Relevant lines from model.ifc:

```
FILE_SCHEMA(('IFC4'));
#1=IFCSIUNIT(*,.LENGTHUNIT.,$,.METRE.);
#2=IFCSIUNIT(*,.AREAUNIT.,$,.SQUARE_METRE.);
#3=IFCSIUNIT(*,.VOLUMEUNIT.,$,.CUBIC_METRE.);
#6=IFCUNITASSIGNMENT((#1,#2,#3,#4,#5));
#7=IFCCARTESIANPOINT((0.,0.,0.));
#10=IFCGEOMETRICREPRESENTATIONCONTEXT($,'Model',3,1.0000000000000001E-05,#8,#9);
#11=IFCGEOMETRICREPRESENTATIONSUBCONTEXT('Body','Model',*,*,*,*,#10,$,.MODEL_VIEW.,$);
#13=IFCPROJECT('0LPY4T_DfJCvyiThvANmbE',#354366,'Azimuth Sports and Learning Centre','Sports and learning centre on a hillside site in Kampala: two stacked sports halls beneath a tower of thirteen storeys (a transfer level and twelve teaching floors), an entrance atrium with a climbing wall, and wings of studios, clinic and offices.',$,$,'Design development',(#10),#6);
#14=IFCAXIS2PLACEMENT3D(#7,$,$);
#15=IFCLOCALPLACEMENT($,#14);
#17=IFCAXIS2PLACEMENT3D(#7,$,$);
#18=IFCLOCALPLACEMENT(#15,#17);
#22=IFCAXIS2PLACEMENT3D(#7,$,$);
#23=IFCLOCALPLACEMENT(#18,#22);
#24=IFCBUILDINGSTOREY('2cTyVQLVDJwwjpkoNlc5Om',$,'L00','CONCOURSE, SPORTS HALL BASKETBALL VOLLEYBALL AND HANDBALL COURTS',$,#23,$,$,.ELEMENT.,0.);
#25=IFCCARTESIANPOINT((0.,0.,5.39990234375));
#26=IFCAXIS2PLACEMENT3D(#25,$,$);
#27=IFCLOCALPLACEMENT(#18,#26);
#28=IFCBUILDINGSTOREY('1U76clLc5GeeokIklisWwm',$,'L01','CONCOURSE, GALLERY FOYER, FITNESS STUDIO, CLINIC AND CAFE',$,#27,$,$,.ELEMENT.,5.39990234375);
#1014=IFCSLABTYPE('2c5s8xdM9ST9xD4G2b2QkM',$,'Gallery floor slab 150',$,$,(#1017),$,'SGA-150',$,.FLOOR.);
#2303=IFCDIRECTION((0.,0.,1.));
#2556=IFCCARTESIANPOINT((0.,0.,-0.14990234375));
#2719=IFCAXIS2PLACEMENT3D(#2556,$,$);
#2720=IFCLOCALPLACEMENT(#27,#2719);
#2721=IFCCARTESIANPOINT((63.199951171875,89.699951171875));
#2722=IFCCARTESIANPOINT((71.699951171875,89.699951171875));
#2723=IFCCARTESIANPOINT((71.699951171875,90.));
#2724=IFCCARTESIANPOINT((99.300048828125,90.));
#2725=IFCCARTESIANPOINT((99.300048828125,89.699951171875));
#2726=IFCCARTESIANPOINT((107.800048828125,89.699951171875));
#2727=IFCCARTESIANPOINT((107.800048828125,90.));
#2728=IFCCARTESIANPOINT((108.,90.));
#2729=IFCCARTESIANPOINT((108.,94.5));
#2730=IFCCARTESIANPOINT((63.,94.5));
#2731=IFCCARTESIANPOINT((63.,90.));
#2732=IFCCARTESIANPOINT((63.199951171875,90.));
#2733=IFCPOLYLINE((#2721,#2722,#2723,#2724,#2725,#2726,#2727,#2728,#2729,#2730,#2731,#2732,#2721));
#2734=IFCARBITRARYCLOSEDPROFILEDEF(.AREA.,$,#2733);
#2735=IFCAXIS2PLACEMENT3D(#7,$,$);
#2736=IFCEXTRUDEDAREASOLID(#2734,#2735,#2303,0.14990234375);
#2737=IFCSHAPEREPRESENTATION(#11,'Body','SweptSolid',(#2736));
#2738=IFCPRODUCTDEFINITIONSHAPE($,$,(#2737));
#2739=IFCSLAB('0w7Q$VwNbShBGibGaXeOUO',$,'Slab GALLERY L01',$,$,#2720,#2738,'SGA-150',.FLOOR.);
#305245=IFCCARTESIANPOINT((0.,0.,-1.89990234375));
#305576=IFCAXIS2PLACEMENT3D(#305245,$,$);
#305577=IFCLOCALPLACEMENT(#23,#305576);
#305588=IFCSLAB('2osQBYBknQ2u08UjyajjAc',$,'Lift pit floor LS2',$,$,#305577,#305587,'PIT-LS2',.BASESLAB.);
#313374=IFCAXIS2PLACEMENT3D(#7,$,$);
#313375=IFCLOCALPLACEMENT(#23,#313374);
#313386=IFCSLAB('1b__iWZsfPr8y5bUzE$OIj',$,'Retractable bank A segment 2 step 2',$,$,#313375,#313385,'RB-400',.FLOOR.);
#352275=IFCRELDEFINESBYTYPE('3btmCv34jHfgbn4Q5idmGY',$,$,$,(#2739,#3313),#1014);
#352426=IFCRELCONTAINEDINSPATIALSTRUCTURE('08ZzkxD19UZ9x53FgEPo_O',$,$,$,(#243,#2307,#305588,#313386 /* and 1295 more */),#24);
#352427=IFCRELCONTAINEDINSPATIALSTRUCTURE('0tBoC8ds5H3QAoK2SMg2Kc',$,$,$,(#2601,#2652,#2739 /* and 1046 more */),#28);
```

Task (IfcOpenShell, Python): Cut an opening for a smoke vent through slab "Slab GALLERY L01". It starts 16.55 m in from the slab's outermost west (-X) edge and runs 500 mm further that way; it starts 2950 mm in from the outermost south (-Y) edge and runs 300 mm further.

```python
import numpy as np
import ifcopenshell
import ifcopenshell.api.feature
import ifcopenshell.api.geometry
import ifcopenshell.api.root
import ifcopenshell.geom
import ifcopenshell.util.placement
import ifcopenshell.util.representation
import ifcopenshell.util.shape
import ifcopenshell.util.unit

model = ifcopenshell.open("model.ifc")
unit_scale = ifcopenshell.util.unit.calculate_unit_scale(model)
settings = ifcopenshell.geom.settings()


def volume(element):
    """Net volume in cubic metres, openings subtracted."""
    shape = ifcopenshell.geom.create_shape(settings, element)
    return ifcopenshell.util.shape.get_volume(shape.geometry)


slab = model.by_guid("0w7Q$VwNbShBGibGaXeOUO")
before = volume(slab)

# Extent in the slab's own axes, in metres. The edges named are its -X and -Y sides.
slab_shape = ifcopenshell.geom.create_shape(settings, slab)
vertices = ifcopenshell.util.shape.get_vertices(slab_shape.geometry)
x_min, y_min, bottom = vertices.min(axis=0)
top = vertices[:, 2].max()

opening = ifcopenshell.api.root.create_entity(model, ifc_class="IfcOpeningElement", name="Smoke vent opening", predefined_type="OPENING")
context = ifcopenshell.util.representation.get_context(model, "Model", "Body", "MODEL_VIEW")
width, depth = 0.5, 0.3
outline = [(0.0, 0.0), (width, 0.0), (width, depth), (0.0, depth), (0.0, 0.0)]
# Overshoot both faces by 50 mm so the cut is clean.
shape = ifcopenshell.api.geometry.add_slab_representation(
    model, context=context, depth=top - bottom + 0.1, polyline=outline
)
ifcopenshell.api.geometry.assign_representation(model, product=opening, representation=shape)

matrix = ifcopenshell.util.placement.get_local_placement(slab.ObjectPlacement)
matrix[:, 3] = matrix @ np.append(np.array([x_min + 16.55, y_min + 2.95, bottom - 0.05]) / unit_scale, 1.0)
ifcopenshell.api.geometry.edit_object_placement(model, product=opening, matrix=matrix, is_si=False)
ifcopenshell.api.feature.add_feature(model, feature=opening, element=slab)

after = volume(slab)

print(f"slab volume {before:.3f} -> {after:.3f} m3")

model.write("model-out.ifc")
```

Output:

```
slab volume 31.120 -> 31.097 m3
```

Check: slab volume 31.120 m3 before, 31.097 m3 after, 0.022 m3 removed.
